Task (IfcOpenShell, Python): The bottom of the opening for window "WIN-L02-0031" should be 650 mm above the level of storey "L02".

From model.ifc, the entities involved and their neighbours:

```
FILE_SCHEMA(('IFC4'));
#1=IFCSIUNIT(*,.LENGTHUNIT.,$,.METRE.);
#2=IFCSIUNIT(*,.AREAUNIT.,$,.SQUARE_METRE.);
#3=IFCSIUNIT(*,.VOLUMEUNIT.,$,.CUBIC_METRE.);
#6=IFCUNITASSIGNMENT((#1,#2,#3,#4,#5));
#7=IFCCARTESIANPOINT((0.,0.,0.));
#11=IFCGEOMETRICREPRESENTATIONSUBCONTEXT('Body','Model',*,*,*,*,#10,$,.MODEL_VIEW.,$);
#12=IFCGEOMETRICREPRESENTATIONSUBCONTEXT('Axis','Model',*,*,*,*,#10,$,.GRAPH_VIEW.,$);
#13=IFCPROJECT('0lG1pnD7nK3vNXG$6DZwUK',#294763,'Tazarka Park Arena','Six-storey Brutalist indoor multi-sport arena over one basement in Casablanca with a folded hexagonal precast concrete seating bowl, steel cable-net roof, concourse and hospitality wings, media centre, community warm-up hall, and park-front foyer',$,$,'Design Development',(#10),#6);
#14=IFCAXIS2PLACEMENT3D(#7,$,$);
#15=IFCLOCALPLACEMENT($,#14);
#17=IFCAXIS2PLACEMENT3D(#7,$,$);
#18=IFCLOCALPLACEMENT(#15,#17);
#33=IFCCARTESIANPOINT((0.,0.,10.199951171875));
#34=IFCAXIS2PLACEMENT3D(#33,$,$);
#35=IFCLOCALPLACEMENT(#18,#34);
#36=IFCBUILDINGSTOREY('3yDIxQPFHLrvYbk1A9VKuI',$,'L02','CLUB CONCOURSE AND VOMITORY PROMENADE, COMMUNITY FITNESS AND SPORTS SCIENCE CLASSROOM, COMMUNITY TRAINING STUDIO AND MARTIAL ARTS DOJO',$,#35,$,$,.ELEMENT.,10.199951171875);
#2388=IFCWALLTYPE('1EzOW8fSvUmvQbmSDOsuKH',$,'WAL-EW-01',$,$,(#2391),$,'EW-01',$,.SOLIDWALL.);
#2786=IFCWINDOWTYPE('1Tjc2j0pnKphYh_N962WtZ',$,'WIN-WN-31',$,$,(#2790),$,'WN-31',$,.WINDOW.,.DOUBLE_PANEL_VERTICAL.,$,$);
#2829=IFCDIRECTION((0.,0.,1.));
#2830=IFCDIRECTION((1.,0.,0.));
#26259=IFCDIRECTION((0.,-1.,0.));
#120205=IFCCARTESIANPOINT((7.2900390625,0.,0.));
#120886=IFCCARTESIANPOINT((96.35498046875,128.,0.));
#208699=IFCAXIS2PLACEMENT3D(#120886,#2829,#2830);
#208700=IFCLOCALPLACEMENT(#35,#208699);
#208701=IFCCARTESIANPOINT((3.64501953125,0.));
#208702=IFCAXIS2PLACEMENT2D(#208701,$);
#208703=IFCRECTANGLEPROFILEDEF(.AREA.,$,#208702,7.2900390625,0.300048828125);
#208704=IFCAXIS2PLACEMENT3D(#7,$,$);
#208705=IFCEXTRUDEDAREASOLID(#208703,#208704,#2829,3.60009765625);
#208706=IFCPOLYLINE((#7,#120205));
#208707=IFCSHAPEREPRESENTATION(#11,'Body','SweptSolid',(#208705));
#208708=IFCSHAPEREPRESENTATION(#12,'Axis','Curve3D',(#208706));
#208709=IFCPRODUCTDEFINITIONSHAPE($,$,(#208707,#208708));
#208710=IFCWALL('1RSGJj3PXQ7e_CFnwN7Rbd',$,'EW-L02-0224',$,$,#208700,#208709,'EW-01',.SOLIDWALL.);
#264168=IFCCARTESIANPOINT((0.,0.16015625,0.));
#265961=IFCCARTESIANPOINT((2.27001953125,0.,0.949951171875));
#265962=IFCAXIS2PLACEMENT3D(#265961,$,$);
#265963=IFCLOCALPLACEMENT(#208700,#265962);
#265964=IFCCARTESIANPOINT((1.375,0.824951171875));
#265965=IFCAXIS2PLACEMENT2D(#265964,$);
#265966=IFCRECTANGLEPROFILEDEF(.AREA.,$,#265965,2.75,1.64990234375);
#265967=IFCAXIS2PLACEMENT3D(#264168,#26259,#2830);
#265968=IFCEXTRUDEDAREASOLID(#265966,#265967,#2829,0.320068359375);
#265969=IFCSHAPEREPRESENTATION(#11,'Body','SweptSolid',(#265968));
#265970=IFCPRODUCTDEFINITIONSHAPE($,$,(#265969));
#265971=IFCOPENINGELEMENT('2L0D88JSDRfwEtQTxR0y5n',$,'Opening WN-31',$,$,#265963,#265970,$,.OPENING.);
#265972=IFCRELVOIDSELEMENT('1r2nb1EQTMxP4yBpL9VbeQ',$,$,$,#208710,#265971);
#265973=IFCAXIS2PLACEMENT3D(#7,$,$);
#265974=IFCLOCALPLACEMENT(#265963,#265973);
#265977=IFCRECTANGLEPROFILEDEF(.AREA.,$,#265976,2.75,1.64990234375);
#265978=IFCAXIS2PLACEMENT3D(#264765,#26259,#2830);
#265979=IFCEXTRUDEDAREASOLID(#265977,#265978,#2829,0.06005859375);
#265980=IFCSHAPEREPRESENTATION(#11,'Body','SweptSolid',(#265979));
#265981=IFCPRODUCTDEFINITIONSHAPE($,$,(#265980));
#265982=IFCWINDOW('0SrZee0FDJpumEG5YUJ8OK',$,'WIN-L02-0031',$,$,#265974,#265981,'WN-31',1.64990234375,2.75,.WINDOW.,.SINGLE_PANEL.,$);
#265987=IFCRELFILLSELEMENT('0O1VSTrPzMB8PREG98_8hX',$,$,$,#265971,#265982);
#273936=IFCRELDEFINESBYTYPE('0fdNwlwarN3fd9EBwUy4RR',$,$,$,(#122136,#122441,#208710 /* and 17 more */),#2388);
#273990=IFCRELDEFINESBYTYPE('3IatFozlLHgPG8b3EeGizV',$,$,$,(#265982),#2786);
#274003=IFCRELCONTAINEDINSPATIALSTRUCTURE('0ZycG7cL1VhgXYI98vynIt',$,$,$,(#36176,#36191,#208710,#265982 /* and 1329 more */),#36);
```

```python
import numpy as np
import ifcopenshell
import ifcopenshell.api.geometry
import ifcopenshell.geom
import ifcopenshell.util.element
import ifcopenshell.util.placement
import ifcopenshell.util.shape
import ifcopenshell.util.unit

model = ifcopenshell.open("model.ifc")
unit_scale = ifcopenshell.util.unit.calculate_unit_scale(model)

window = model.by_id(265982)
opening = window.FillsVoids[0].RelatingOpeningElement
storey = ifcopenshell.util.element.get_container(window, ifc_class="IfcBuildingStorey")
level = ifcopenshell.util.placement.get_local_placement(storey.ObjectPlacement)[2, 3]

# The opening's origin need not be at the sill, so measure its lowest point.
shape = ifcopenshell.geom.create_shape(ifcopenshell.geom.settings(), opening)
bottom = ifcopenshell.util.shape.get_shape_bottom_elevation(shape, shape.geometry) / unit_scale
dz = level + 0.65 / unit_scale - bottom

shift = np.array([0.0, 0.0, dz])
# The window is placed relative to its opening, so it follows when the opening moves.
matrix = ifcopenshell.util.placement.get_local_placement(opening.ObjectPlacement)
matrix[:3, 3] += shift
ifcopenshell.api.geometry.edit_object_placement(
    model, product=opening, matrix=matrix, is_si=False, should_transform_children=True
)

print(f"moved by {dz * unit_scale:+.3f} m")

model.write("model_rev.ifc")
```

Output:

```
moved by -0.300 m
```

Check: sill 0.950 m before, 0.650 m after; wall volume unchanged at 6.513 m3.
